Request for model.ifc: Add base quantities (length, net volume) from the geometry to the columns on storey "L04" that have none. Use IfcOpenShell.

First a look at what the model holds.

```python
import ifcopenshell
import ifcopenshell.util.element
import ifcopenshell.util.unit

model = ifcopenshell.open("model.ifc")
print(model.schema)
for unit_type in ("LENGTHUNIT", "AREAUNIT", "VOLUMEUNIT"):
    print(unit_type, ifcopenshell.util.unit.calculate_unit_scale(model, unit_type))
storey = next(s for s in model.by_type("IfcBuildingStorey") if s.Name == "L04")
columns = [e for e in ifcopenshell.util.element.get_decomposition(storey) if e.is_a("IfcColumn")]
for e in sorted(columns, key=lambda e: e.id()):
    print(e.id(), e.is_a(), e.Name, list(ifcopenshell.util.element.get_psets(e, qtos_only=True)), sep=" | ")
```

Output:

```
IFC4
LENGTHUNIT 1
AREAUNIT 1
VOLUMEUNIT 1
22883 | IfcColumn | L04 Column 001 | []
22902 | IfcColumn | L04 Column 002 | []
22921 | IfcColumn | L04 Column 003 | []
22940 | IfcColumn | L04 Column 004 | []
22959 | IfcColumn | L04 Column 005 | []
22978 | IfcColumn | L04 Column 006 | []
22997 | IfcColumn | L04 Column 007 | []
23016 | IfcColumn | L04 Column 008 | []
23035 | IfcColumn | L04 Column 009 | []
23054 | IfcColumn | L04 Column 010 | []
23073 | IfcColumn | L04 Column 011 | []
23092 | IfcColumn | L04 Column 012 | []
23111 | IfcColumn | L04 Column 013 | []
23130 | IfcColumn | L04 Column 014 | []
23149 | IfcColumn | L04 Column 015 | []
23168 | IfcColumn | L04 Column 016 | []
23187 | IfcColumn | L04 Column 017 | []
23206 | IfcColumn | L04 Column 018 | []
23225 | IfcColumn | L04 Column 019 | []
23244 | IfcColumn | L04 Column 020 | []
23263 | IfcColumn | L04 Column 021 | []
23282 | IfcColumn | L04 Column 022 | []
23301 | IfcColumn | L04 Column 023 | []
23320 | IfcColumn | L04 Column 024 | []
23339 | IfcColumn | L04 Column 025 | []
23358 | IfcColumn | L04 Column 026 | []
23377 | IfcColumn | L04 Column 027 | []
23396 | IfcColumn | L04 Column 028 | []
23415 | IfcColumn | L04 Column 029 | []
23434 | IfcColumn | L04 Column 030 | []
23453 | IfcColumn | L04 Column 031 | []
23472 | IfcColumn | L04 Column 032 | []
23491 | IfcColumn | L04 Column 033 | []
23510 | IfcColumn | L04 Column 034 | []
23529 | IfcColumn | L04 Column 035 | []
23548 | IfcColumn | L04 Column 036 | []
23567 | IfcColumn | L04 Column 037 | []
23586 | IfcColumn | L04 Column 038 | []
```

```python
import ifcopenshell
import ifcopenshell.api.pset
import ifcopenshell.geom
import ifcopenshell.util.element
import ifcopenshell.util.shape
import ifcopenshell.util.unit

model = ifcopenshell.open("model.ifc")
unit_scale = ifcopenshell.util.unit.calculate_unit_scale(model)
volume_scale = ifcopenshell.util.unit.calculate_unit_scale(model, "VOLUMEUNIT")
settings = ifcopenshell.geom.settings()

storey = next(s for s in model.by_type("IfcBuildingStorey") if s.Name == "L04")
columns = [e for e in ifcopenshell.util.element.get_decomposition(storey) if e.is_a("IfcColumn")]

for e in sorted(columns, key=lambda e: e.id()):
    if ifcopenshell.util.element.get_psets(e, qtos_only=True, should_inherit=False):
        continue
    # Geometry comes back in metres, in the element's own axes.
    shape = ifcopenshell.geom.create_shape(settings, e)
    values = {
        "Length": ifcopenshell.util.shape.get_z(shape.geometry) / unit_scale,
        "NetVolume": ifcopenshell.util.shape.get_volume(shape.geometry) / volume_scale,
    }
    qto = ifcopenshell.api.pset.add_qto(model, product=e, name="Qto_ColumnBaseQuantities")
    ifcopenshell.api.pset.edit_qto(model, qto=qto, properties=values)
    print(e.id(), {k: round(v, 3) for k, v in values.items()})

model.write("model-out.ifc")
```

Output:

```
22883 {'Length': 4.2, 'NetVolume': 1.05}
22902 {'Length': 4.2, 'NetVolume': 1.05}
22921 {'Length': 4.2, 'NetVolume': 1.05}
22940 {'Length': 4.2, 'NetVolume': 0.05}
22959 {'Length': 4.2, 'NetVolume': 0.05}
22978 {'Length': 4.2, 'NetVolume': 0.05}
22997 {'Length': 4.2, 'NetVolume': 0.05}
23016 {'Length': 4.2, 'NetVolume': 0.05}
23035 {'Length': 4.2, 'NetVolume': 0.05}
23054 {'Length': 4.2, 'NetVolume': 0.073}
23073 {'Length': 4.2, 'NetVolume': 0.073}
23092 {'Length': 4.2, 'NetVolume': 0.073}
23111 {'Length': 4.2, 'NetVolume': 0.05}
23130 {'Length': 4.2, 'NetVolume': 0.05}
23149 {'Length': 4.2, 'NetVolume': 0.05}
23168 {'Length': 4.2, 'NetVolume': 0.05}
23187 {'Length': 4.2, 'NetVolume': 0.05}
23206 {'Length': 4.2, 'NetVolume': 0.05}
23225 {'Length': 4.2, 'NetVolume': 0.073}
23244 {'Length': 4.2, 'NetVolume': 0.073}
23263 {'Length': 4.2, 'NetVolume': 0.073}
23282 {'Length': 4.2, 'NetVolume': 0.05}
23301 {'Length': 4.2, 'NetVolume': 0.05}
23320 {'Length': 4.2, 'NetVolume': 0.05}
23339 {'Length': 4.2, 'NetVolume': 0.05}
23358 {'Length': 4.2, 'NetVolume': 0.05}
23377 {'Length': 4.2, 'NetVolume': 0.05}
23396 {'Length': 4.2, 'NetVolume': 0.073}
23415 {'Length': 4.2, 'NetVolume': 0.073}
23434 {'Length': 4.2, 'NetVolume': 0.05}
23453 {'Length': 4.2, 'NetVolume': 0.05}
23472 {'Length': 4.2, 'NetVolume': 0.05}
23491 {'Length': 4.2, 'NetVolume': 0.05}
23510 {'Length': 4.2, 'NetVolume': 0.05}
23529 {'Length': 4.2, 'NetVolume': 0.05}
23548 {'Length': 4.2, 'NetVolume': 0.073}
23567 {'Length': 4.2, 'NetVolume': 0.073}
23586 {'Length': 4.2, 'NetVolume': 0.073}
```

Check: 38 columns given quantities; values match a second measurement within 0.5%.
